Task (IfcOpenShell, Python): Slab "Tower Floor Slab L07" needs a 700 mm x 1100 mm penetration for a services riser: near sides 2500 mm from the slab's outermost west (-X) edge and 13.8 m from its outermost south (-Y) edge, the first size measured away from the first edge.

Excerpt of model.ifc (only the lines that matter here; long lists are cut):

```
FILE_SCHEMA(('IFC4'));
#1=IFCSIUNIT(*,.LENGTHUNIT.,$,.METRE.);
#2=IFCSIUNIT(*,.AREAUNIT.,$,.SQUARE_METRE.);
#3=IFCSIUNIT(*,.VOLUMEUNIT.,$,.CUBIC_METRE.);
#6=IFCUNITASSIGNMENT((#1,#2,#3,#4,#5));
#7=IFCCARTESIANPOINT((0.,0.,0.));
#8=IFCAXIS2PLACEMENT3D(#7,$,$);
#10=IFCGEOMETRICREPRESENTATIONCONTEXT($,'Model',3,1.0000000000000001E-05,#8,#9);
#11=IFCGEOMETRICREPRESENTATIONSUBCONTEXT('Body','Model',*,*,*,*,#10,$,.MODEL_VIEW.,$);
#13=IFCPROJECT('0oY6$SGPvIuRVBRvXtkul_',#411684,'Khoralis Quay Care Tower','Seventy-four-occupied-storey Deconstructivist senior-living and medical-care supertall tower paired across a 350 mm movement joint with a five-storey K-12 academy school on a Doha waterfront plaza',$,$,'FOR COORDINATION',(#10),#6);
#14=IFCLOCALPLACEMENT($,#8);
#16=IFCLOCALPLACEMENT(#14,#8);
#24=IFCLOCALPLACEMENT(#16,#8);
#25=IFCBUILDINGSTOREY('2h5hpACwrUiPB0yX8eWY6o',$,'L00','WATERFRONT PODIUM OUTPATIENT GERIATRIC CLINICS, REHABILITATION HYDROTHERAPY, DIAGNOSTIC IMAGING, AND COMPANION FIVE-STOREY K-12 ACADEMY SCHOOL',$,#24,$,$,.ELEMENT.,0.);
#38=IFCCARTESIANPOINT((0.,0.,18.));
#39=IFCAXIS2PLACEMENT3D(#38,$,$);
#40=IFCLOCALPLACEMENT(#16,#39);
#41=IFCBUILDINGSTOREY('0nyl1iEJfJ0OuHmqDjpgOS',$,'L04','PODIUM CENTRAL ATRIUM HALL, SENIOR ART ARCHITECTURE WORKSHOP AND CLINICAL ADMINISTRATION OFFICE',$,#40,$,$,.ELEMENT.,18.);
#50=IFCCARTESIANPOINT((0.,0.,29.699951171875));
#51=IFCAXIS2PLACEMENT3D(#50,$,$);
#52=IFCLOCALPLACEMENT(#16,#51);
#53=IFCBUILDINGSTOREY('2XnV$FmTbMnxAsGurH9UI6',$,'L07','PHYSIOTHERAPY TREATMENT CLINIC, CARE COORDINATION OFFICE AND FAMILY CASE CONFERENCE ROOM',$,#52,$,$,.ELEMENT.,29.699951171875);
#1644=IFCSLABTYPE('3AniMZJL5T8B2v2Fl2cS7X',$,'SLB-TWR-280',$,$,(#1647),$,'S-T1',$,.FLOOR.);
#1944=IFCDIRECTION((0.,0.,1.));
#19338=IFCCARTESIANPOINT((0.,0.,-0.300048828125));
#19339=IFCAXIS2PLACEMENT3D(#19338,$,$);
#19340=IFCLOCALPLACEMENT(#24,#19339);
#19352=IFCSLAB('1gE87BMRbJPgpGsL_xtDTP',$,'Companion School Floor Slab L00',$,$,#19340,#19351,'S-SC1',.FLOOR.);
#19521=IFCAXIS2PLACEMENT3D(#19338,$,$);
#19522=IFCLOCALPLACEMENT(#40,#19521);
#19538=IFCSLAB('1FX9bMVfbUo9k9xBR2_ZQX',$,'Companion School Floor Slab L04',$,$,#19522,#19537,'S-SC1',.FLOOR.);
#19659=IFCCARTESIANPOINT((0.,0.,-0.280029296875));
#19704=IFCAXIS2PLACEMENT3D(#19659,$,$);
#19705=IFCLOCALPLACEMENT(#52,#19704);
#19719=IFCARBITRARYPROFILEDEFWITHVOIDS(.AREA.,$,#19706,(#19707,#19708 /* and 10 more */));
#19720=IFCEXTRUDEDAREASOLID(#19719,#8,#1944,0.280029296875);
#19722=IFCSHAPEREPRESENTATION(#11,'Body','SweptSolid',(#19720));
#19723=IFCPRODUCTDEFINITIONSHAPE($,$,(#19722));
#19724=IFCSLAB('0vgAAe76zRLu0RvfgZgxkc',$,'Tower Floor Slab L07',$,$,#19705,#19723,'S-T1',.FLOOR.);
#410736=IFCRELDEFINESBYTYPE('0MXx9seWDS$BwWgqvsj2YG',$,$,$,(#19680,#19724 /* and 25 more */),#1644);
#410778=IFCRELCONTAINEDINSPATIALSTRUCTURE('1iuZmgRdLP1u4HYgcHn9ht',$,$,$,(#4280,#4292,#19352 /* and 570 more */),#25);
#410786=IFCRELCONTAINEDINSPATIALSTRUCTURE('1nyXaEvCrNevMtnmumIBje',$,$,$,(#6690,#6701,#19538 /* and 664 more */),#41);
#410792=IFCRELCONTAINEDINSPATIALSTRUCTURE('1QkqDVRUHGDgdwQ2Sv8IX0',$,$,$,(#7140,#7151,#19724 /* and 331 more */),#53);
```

```python
import numpy as np
import ifcopenshell
import ifcopenshell.api.feature
import ifcopenshell.api.geometry
import ifcopenshell.api.root
import ifcopenshell.geom
import ifcopenshell.util.placement
import ifcopenshell.util.representation
import ifcopenshell.util.shape
import ifcopenshell.util.unit

model = ifcopenshell.open("model.ifc")
unit_scale = ifcopenshell.util.unit.calculate_unit_scale(model)
settings = ifcopenshell.geom.settings()


def volume(element):
    """Net volume in cubic metres, openings subtracted."""
    shape = ifcopenshell.geom.create_shape(settings, element)
    return ifcopenshell.util.shape.get_volume(shape.geometry)


slab = model.by_guid("0vgAAe76zRLu0RvfgZgxkc")
before = volume(slab)

# Extent in the slab's own axes, in metres. The edges named are its -X and -Y sides.
slab_shape = ifcopenshell.geom.create_shape(settings, slab)
vertices = ifcopenshell.util.shape.get_vertices(slab_shape.geometry)
x_min, y_min, bottom = vertices.min(axis=0)
top = vertices[:, 2].max()

opening = ifcopenshell.api.root.create_entity(model, ifc_class="IfcOpeningElement", name="Services riser opening", predefined_type="OPENING")
context = ifcopenshell.util.representation.get_context(model, "Model", "Body", "MODEL_VIEW")
width, depth = 0.7, 1.1
outline = [(0.0, 0.0), (width, 0.0), (width, depth), (0.0, depth), (0.0, 0.0)]
# Overshoot both faces by 50 mm so the cut is clean.
shape = ifcopenshell.api.geometry.add_slab_representation(
    model, context=context, depth=top - bottom + 0.1, polyline=outline
)
ifcopenshell.api.geometry.assign_representation(model, product=opening, representation=shape)

matrix = ifcopenshell.util.placement.get_local_placement(slab.ObjectPlacement)
matrix[:, 3] = matrix @ np.append(np.array([x_min + 2.5, y_min + 13.8, bottom - 0.05]) / unit_scale, 1.0)
ifcopenshell.api.geometry.edit_object_placement(model, product=opening, matrix=matrix, is_si=False)
ifcopenshell.api.feature.add_feature(model, feature=opening, element=slab)

after = volume(slab)

print(f"slab volume {before:.3f} -> {after:.3f} m3")

model.write("model_updated.ifc")
```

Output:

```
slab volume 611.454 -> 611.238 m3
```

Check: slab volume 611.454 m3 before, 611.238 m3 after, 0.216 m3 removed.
